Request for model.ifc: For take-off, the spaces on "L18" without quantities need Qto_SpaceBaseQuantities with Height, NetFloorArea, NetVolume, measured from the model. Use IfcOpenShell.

First a look at what the model holds.

```python
import ifcopenshell
import ifcopenshell.util.element
import ifcopenshell.util.unit

model = ifcopenshell.open("model.ifc")
print(model.schema)
for unit_type in ("LENGTHUNIT", "AREAUNIT", "VOLUMEUNIT"):
    print(unit_type, ifcopenshell.util.unit.calculate_unit_scale(model, unit_type))
storey = next(s for s in model.by_type("IfcBuildingStorey") if s.Name == "L18")
spaces = [e for e in ifcopenshell.util.element.get_decomposition(storey) if e.is_a("IfcSpace")]
for e in sorted(spaces, key=lambda e: e.id()):
    print(e.id(), e.is_a(), e.Name, list(ifcopenshell.util.element.get_psets(e, qtos_only=True)), sep=" | ")
```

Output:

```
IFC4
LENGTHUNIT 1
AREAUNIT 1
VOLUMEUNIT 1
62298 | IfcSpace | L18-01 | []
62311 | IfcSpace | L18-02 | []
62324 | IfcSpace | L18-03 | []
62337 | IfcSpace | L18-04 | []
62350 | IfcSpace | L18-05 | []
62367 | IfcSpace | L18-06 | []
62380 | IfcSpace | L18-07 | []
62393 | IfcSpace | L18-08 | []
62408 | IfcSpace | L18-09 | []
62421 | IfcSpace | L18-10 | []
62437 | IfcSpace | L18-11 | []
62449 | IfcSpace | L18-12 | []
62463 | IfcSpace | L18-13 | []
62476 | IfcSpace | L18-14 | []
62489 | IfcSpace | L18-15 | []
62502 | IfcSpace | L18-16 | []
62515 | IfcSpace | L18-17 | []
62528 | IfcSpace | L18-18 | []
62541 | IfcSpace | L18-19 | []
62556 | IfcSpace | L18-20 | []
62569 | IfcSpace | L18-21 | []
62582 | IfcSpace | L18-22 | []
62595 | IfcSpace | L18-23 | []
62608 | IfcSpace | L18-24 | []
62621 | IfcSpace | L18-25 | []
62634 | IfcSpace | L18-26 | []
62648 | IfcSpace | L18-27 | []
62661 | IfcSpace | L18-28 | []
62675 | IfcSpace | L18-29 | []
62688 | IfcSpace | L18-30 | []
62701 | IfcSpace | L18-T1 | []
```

```python
import ifcopenshell
import ifcopenshell.api.pset
import ifcopenshell.geom
import ifcopenshell.util.element
import ifcopenshell.util.shape
import ifcopenshell.util.unit

model = ifcopenshell.open("model.ifc")
unit_scale = ifcopenshell.util.unit.calculate_unit_scale(model)
area_scale = ifcopenshell.util.unit.calculate_unit_scale(model, "AREAUNIT")
volume_scale = ifcopenshell.util.unit.calculate_unit_scale(model, "VOLUMEUNIT")
settings = ifcopenshell.geom.settings()

storey = next(s for s in model.by_type("IfcBuildingStorey") if s.Name == "L18")
spaces = [e for e in ifcopenshell.util.element.get_decomposition(storey) if e.is_a("IfcSpace")]

for e in sorted(spaces, key=lambda e: e.id()):
    if ifcopenshell.util.element.get_psets(e, qtos_only=True, should_inherit=False):
        continue
    # Geometry comes back in metres, in the element's own axes.
    shape = ifcopenshell.geom.create_shape(settings, e)
    values = {
        "Height": ifcopenshell.util.shape.get_z(shape.geometry) / unit_scale,
        "NetFloorArea": ifcopenshell.util.shape.get_footprint_area(shape.geometry) / area_scale,
        "NetVolume": ifcopenshell.util.shape.get_volume(shape.geometry) / volume_scale,
    }
    qto = ifcopenshell.api.pset.add_qto(model, product=e, name="Qto_SpaceBaseQuantities")
    ifcopenshell.api.pset.edit_qto(model, qto=qto, properties=values)
    print(e.id(), {k: round(v, 3) for k, v in values.items()})

model.write("model_updated.ifc")
```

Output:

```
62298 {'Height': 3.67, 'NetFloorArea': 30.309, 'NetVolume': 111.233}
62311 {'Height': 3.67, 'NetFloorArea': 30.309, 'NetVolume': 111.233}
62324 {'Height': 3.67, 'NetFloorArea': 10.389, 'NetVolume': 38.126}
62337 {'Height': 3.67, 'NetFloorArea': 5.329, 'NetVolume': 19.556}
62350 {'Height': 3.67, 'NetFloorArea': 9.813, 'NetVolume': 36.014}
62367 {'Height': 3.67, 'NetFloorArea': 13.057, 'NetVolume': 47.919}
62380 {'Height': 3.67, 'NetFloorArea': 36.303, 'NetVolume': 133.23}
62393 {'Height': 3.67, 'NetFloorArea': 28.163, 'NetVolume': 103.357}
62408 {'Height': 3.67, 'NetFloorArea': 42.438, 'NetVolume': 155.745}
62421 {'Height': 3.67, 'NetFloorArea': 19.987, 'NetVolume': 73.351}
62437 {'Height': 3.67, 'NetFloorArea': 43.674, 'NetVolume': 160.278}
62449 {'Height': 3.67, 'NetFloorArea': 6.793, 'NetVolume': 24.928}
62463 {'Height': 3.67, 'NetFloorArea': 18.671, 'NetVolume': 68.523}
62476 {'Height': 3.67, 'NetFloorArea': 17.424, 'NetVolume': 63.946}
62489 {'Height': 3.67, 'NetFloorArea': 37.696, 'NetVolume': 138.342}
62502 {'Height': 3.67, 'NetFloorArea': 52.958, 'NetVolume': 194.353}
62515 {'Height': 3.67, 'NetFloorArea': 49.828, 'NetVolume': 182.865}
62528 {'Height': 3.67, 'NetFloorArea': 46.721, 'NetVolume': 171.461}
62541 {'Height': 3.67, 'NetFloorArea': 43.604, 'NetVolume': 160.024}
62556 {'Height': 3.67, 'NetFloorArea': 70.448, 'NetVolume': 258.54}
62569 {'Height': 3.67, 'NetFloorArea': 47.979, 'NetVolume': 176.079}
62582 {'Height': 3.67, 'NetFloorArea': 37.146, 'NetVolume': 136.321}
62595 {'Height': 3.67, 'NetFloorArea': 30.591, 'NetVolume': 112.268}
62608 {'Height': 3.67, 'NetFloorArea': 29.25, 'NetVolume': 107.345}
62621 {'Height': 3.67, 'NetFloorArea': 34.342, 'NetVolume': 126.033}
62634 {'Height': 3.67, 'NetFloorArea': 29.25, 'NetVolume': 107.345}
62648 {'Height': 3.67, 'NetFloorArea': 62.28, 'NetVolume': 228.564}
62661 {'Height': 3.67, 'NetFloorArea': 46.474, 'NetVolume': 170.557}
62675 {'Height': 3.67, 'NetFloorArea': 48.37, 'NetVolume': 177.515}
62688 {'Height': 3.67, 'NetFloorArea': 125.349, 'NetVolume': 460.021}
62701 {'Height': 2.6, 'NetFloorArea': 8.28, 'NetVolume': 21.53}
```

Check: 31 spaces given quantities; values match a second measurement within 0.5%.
